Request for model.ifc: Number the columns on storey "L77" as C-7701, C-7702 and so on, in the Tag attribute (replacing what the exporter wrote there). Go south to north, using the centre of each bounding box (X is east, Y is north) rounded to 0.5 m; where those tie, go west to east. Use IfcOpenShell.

First a look at what the model holds.

```python
import ifcopenshell
import ifcopenshell.util.element
import ifcopenshell.util.placement

model = ifcopenshell.open("model.ifc")
print(model.schema)
storey = next(s for s in model.by_type("IfcBuildingStorey") if s.Name == "L77")
columns = [e for e in ifcopenshell.util.element.get_decomposition(storey) if e.is_a("IfcColumn")]
for e in sorted(columns, key=lambda e: e.id()):
    origin = ifcopenshell.util.placement.get_local_placement(e.ObjectPlacement)[:3, 3]
    print(e.id(), e.Tag, e.Name, origin.round(2) + 0.0, sep=" | ")
```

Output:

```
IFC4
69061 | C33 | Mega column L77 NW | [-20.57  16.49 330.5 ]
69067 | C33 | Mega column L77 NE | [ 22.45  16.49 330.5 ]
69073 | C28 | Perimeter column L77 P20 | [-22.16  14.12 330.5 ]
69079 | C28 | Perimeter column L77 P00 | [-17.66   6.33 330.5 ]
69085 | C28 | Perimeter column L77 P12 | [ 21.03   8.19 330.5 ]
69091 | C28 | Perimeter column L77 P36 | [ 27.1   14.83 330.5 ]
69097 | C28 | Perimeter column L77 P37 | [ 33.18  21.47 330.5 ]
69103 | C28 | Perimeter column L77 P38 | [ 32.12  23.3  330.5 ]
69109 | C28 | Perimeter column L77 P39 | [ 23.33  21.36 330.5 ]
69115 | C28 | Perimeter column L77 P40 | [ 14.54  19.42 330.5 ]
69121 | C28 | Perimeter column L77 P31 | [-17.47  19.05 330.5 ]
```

```python
import ifcopenshell
import ifcopenshell.geom
import ifcopenshell.util.element
import ifcopenshell.util.shape

model = ifcopenshell.open("model.ifc")
settings = ifcopenshell.geom.settings()
settings.set("use-world-coords", True)


def centre(element):
    shape = ifcopenshell.geom.create_shape(settings, element)
    return ifcopenshell.util.shape.get_bbox_centroid(shape.geometry)


storey = next(s for s in model.by_type("IfcBuildingStorey") if s.Name == "L77")
columns = [e for e in ifcopenshell.util.element.get_decomposition(storey) if e.is_a("IfcColumn")]

# Insertion points can sit at a corner or the storey origin, so sort by the geometry (in metres).
centres = {e: centre(e) for e in columns}
columns.sort(key=lambda e: (round(centres[e][1] / 0.5), centres[e][0]))

for i, e in enumerate(columns, start=1):
    number = f"C-77{i:02d}"
    e.Tag = number
    print(e.id(), number)

model.write("model_edited.ifc")
```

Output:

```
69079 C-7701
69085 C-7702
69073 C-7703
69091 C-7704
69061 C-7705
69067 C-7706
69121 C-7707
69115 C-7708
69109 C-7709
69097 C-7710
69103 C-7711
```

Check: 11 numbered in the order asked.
